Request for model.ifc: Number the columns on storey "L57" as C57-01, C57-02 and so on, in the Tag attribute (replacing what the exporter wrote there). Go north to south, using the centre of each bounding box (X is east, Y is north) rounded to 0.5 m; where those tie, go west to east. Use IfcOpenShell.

First a look at what the model holds.

```python
import ifcopenshell
import ifcopenshell.util.element
import ifcopenshell.util.placement

model = ifcopenshell.open("model.ifc")
print(model.schema)
storey = next(s for s in model.by_type("IfcBuildingStorey") if s.Name == "L57")
columns = [e for e in ifcopenshell.util.element.get_decomposition(storey) if e.is_a("IfcColumn")]
for e in sorted(columns, key=lambda e: e.id()):
    origin = ifcopenshell.util.placement.get_local_placement(e.ObjectPlacement)[:3, 3]
    print(e.id(), e.Tag, e.Name, origin.round(2) + 0.0, sep=" | ")
```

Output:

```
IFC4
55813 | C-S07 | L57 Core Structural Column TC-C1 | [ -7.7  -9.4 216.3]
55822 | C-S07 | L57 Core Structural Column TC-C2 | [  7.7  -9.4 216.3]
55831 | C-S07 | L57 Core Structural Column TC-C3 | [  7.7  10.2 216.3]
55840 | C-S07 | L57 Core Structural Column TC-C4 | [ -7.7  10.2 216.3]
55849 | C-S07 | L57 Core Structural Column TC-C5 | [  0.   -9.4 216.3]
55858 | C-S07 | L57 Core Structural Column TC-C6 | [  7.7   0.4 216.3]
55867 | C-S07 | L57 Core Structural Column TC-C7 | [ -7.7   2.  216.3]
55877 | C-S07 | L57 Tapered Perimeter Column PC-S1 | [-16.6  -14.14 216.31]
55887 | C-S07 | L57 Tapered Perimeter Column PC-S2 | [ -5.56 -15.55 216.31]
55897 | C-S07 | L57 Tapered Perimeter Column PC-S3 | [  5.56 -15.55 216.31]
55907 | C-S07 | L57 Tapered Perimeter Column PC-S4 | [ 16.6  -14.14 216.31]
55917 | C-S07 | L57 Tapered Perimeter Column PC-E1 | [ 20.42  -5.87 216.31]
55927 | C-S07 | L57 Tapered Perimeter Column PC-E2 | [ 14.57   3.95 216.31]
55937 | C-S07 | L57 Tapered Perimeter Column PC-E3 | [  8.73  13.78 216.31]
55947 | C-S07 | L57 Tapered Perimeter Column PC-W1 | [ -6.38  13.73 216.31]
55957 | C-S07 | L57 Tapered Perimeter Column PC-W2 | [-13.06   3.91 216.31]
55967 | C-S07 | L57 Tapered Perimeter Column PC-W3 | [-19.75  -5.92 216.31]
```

```python
import ifcopenshell
import ifcopenshell.geom
import ifcopenshell.util.element
import ifcopenshell.util.shape

model = ifcopenshell.open("model.ifc")
settings = ifcopenshell.geom.settings()
settings.set("use-world-coords", True)


def centre(element):
    shape = ifcopenshell.geom.create_shape(settings, element)
    return ifcopenshell.util.shape.get_bbox_centroid(shape.geometry)


storey = next(s for s in model.by_type("IfcBuildingStorey") if s.Name == "L57")
columns = [e for e in ifcopenshell.util.element.get_decomposition(storey) if e.is_a("IfcColumn")]

# Insertion points can sit at a corner or the storey origin, so sort by the geometry (in metres).
centres = {e: centre(e) for e in columns}
columns.sort(key=lambda e: (-round(centres[e][1] / 0.5), centres[e][0]))

for i, e in enumerate(columns, start=1):
    number = f"C57-{i:02d}"
    e.Tag = number
    print(e.id(), number)

model.write("model_v2.ifc")
```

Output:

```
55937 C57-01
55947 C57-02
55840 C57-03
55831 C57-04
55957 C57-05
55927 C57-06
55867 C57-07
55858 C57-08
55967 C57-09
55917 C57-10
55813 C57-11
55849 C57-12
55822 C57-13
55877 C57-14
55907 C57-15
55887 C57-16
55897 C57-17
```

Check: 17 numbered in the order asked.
